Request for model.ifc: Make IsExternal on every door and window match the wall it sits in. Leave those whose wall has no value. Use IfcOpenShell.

First a look at what the model holds.

```python
import ifcopenshell
import ifcopenshell.util.element

model = ifcopenshell.open("model.ifc")
print(model.schema)
seen = {}
for e in model.by_type("IfcDoor") + model.by_type("IfcWindow"):
    if not e.FillsVoids:
        continue
    host = e.FillsVoids[0].RelatingOpeningElement.VoidsElements[0].RelatingBuildingElement
    own = ifcopenshell.util.element.get_pset(e, f"Pset_{e.is_a()[3:].removesuffix('StandardCase')}Common", "IsExternal")
    wall = ifcopenshell.util.element.get_pset(host, "Pset_WallCommon", "IsExternal")
    seen[e.is_a(), own, wall] = seen.get((e.is_a(), own, wall), 0) + 1
for (cls, own, wall), count in sorted(seen.items(), key=str):
    print(count, cls, "IsExternal:", own, "| host wall:", wall)
```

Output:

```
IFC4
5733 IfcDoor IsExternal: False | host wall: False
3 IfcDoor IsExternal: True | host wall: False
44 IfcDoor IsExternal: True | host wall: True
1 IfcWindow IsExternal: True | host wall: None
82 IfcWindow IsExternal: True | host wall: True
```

```python
import ifcopenshell
import ifcopenshell.api.pset
import ifcopenshell.util.element

model = ifcopenshell.open("model.ifc")

count = 0
for ifc_class, pset_name in (("IfcDoor", "Pset_DoorCommon"), ("IfcWindow", "Pset_WindowCommon")):
    for e in model.by_type(ifc_class):
        if not e.FillsVoids:
            continue
        host = e.FillsVoids[0].RelatingOpeningElement.VoidsElements[0].RelatingBuildingElement
        external = ifcopenshell.util.element.get_pset(host, "Pset_WallCommon", "IsExternal")
        if external is None or ifcopenshell.util.element.get_pset(e, pset_name, "IsExternal") == external:
            continue
        found = ifcopenshell.util.element.get_pset(e, pset_name, should_inherit=False)
        if found:
            pset = model.by_id(found["id"])
            if len(ifcopenshell.util.element.get_elements_by_pset(pset)) > 1:
                pset = ifcopenshell.api.pset.unshare_pset(model, products=[e], pset=pset)[0]
        else:
            pset = ifcopenshell.api.pset.add_pset(model, product=e, name=pset_name)
        ifcopenshell.api.pset.edit_pset(model, pset=pset, properties={"IsExternal": external})
        count += 1

print(count, "updated")

model.write("model_updated.ifc")
```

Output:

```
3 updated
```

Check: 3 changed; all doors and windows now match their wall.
